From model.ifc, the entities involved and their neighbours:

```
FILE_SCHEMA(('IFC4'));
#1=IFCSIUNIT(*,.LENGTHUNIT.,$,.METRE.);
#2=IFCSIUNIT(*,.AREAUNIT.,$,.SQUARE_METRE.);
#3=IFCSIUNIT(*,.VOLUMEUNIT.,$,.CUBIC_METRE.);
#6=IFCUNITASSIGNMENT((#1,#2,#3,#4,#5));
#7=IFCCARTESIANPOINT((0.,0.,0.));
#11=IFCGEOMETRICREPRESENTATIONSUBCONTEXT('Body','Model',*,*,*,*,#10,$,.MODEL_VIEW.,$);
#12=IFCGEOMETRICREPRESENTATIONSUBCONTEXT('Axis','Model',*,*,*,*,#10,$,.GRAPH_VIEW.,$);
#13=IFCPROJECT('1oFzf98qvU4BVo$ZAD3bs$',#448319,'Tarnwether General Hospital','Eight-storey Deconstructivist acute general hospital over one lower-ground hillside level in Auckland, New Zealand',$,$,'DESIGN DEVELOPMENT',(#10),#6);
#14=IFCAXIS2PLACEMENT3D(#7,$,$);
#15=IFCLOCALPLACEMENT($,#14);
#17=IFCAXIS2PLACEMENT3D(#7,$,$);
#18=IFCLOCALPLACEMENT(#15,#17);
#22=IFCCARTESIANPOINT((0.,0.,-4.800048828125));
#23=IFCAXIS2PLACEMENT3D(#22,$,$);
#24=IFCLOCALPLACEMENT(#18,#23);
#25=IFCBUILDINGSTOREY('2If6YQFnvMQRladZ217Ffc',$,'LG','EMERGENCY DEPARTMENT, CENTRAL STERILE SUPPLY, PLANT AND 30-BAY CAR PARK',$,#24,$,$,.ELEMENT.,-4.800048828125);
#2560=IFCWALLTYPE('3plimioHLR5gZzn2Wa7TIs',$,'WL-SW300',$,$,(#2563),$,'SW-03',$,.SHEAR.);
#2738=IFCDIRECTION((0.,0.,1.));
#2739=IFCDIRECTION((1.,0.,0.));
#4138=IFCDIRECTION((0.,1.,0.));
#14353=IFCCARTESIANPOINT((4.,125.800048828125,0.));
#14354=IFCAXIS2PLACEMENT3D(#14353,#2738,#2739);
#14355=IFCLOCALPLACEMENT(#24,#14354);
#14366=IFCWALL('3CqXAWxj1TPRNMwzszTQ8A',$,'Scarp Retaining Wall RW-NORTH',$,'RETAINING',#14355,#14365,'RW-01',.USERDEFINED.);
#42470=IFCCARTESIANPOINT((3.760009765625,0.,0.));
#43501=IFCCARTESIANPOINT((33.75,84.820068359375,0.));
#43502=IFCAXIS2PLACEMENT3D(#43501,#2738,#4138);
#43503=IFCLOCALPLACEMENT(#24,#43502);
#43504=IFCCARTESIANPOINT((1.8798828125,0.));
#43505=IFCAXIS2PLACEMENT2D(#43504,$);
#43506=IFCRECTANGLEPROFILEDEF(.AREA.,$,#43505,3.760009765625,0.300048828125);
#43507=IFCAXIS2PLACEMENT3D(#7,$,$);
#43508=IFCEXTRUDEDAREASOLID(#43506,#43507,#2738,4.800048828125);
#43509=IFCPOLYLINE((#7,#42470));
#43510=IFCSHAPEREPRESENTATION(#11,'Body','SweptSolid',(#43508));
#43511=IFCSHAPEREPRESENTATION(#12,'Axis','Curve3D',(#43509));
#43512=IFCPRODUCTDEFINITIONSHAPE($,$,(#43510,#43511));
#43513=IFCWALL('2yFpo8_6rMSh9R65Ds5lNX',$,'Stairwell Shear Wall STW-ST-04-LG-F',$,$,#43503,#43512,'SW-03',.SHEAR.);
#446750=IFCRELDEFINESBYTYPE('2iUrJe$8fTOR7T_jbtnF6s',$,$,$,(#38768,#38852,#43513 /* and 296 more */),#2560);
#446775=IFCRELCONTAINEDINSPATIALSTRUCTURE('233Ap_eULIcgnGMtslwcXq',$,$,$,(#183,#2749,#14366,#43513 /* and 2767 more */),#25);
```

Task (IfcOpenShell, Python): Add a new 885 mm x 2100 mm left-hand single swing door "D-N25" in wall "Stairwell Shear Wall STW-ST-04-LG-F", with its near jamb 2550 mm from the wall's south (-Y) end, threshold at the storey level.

```python
import numpy as np
import ifcopenshell
import ifcopenshell.api.feature
import ifcopenshell.api.geometry
import ifcopenshell.api.root
import ifcopenshell.api.spatial
import ifcopenshell.geom
import ifcopenshell.util.element
import ifcopenshell.util.placement
import ifcopenshell.util.representation
import ifcopenshell.util.shape
import ifcopenshell.util.unit

model = ifcopenshell.open("model.ifc")
unit_scale = ifcopenshell.util.unit.calculate_unit_scale(model)
settings = ifcopenshell.geom.settings()


def volume(element):
    """Net volume in cubic metres, openings subtracted."""
    shape = ifcopenshell.geom.create_shape(settings, element)
    return ifcopenshell.util.shape.get_volume(shape.geometry)


wall = model.by_guid("2yFpo8_6rMSh9R65Ds5lNX")
storey = ifcopenshell.util.element.get_container(wall, ifc_class="IfcBuildingStorey")
context = ifcopenshell.util.representation.get_context(model, "Model", "Body", "MODEL_VIEW")
before = volume(wall)

width, height, from_end, sill = 0.885, 2.1, 2.55, 0.0  # metres

# The wall runs along its own X axis, and the end named is its -X end.
wall_shape = ifcopenshell.geom.create_shape(settings, wall)
x, y, z = ifcopenshell.util.shape.get_vertices(wall_shape.geometry).T
start = x.min() + from_end
face, thickness = float(y.min()), float(y.max() - y.min())
wall_matrix = ifcopenshell.util.placement.get_local_placement(wall.ObjectPlacement)
level = ifcopenshell.util.placement.get_local_placement(storey.ObjectPlacement)[2, 3]


def in_wall(x, y):
    """Placement at x, y metres in the wall's axes, at sill height."""
    matrix = wall_matrix.copy()
    matrix[:, 3] = wall_matrix @ np.array([x / unit_scale, y / unit_scale, 0.0, 1.0])
    matrix[2, 3] = level + sill / unit_scale
    return matrix


# Opening: a box that overshoots both wall faces by 50 mm.
opening = ifcopenshell.api.root.create_entity(model, ifc_class="IfcOpeningElement", predefined_type="OPENING")
box = ifcopenshell.api.geometry.add_wall_representation(
    model, context=context, length=width, height=height, thickness=thickness + 0.1
)
ifcopenshell.api.geometry.assign_representation(model, product=opening, representation=box)
ifcopenshell.api.geometry.edit_object_placement(model, product=opening, matrix=in_wall(start, face - 0.05), is_si=False)
ifcopenshell.api.feature.add_feature(model, feature=opening, element=wall)

door = ifcopenshell.api.root.create_entity(model, ifc_class="IfcDoor", name="D-N25", predefined_type="DOOR")
door.OverallWidth, door.OverallHeight = width / unit_scale, height / unit_scale
door.OperationType = "SINGLE_SWING_LEFT"
body = ifcopenshell.api.geometry.add_door_representation(
    model,
    context=context,
    overall_width=door.OverallWidth,
    overall_height=door.OverallHeight,
    operation_type="SINGLE_SWING_LEFT",
    lining_properties={"LiningDepth": thickness / unit_scale, "ThresholdDepth": thickness / unit_scale},
)
ifcopenshell.api.geometry.assign_representation(model, product=door, representation=body)
ifcopenshell.api.spatial.assign_container(model, products=[door], relating_structure=storey)
ifcopenshell.api.feature.add_filling(model, opening=opening, element=door)

# The lining spans the wall, so the door starts at the wall face.
ifcopenshell.api.geometry.edit_object_placement(model, product=door, matrix=in_wall(start, face), is_si=False)

after = volume(wall)

print(f"wall volume {before:.3f} -> {after:.3f} m3")

model.write("model_updated.ifc")
```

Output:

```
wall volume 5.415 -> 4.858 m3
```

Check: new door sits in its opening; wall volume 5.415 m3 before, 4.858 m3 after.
